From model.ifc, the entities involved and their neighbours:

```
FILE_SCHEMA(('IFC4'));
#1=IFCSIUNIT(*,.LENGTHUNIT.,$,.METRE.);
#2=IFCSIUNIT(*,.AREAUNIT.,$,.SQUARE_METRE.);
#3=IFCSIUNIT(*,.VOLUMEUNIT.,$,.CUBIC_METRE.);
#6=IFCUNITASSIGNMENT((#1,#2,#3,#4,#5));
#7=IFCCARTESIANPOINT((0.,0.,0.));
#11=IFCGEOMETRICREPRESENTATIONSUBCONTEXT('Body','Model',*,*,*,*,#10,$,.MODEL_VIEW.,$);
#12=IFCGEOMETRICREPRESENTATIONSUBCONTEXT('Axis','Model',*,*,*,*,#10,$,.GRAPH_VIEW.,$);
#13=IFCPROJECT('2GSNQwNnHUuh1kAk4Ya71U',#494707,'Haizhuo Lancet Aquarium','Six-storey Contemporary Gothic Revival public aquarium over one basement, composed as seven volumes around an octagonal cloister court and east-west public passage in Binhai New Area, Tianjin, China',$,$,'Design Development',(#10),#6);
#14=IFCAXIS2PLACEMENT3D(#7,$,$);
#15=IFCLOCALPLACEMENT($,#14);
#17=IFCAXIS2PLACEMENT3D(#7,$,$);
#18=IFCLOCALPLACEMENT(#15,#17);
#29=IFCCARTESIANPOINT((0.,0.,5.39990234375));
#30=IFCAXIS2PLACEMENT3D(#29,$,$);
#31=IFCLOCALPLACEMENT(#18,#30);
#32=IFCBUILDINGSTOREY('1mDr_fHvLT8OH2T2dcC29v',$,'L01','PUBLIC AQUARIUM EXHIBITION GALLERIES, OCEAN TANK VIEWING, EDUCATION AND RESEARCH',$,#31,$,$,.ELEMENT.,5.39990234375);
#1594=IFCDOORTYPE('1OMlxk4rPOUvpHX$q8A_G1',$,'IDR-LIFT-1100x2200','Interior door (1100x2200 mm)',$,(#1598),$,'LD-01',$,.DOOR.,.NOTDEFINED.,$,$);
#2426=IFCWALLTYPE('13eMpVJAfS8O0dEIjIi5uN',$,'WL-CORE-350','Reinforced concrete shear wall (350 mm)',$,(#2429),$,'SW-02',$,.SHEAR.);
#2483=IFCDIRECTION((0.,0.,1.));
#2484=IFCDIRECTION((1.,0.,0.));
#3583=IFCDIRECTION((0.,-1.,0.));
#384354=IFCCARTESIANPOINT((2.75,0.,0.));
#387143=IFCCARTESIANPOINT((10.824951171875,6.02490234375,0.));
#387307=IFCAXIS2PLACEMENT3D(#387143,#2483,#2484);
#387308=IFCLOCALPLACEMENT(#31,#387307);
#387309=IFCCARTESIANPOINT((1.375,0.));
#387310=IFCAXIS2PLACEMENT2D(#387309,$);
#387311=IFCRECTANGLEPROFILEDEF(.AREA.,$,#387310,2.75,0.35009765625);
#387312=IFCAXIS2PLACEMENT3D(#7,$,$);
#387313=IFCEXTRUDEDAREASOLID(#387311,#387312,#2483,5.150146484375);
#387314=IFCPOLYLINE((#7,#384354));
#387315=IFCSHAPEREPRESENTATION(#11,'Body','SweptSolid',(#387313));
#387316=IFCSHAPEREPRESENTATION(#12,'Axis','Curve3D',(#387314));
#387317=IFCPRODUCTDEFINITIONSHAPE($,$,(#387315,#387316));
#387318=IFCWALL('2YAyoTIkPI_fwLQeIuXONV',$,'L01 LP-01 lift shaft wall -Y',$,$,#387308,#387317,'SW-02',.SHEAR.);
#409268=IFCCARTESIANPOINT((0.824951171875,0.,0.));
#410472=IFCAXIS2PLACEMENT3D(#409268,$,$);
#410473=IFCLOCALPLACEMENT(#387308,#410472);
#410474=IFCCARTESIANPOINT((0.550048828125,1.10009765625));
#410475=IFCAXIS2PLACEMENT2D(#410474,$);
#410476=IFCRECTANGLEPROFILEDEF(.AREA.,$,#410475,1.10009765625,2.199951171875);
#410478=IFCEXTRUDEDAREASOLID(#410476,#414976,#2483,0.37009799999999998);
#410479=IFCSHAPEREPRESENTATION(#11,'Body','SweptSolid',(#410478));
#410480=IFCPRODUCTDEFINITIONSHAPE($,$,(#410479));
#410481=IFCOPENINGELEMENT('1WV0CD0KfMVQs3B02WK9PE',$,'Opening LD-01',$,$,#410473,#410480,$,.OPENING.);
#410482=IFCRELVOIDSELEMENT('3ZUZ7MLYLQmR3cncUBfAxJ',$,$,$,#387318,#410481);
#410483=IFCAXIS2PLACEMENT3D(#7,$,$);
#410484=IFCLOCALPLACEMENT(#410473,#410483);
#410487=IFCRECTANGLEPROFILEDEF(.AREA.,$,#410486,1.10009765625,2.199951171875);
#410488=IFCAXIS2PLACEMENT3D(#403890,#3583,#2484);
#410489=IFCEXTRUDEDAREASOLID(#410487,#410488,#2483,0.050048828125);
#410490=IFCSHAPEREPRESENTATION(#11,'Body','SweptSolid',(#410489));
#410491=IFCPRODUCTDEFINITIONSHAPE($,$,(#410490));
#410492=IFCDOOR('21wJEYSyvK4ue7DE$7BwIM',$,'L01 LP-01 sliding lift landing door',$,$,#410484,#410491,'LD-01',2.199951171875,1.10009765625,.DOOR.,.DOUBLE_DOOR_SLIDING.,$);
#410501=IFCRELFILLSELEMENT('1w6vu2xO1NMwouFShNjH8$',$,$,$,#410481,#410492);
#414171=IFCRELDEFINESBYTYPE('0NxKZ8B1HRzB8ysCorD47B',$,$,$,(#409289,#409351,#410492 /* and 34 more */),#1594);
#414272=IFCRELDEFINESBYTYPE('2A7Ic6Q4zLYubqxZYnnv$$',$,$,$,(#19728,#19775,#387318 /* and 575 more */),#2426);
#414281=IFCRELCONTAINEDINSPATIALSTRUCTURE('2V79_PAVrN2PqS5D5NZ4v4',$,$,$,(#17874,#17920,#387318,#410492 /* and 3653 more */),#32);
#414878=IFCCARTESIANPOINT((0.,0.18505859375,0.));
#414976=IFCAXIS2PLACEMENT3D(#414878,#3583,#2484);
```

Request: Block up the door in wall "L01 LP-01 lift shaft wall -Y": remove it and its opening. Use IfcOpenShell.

```python
import ifcopenshell
import ifcopenshell.api.feature
import ifcopenshell.api.root
import ifcopenshell.geom
import ifcopenshell.util.shape

model = ifcopenshell.open("model.ifc")
settings = ifcopenshell.geom.settings()


def volume(element):
    """Net volume in cubic metres, openings subtracted."""
    shape = ifcopenshell.geom.create_shape(settings, element)
    return ifcopenshell.util.shape.get_volume(shape.geometry)


door = model.by_guid("21wJEYSyvK4ue7DE$7BwIM")
opening = door.FillsVoids[0].RelatingOpeningElement
wall = opening.VoidsElements[0].RelatingBuildingElement
before = volume(wall)

ifcopenshell.api.root.remove_product(model, product=door)
ifcopenshell.api.feature.remove_feature(model, feature=opening)

after = volume(wall)

print(f"wall volume {before:.3f} -> {after:.3f} m3")

model.write("model_updated.ifc")
```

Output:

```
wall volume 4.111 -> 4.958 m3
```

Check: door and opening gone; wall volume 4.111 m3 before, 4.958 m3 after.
